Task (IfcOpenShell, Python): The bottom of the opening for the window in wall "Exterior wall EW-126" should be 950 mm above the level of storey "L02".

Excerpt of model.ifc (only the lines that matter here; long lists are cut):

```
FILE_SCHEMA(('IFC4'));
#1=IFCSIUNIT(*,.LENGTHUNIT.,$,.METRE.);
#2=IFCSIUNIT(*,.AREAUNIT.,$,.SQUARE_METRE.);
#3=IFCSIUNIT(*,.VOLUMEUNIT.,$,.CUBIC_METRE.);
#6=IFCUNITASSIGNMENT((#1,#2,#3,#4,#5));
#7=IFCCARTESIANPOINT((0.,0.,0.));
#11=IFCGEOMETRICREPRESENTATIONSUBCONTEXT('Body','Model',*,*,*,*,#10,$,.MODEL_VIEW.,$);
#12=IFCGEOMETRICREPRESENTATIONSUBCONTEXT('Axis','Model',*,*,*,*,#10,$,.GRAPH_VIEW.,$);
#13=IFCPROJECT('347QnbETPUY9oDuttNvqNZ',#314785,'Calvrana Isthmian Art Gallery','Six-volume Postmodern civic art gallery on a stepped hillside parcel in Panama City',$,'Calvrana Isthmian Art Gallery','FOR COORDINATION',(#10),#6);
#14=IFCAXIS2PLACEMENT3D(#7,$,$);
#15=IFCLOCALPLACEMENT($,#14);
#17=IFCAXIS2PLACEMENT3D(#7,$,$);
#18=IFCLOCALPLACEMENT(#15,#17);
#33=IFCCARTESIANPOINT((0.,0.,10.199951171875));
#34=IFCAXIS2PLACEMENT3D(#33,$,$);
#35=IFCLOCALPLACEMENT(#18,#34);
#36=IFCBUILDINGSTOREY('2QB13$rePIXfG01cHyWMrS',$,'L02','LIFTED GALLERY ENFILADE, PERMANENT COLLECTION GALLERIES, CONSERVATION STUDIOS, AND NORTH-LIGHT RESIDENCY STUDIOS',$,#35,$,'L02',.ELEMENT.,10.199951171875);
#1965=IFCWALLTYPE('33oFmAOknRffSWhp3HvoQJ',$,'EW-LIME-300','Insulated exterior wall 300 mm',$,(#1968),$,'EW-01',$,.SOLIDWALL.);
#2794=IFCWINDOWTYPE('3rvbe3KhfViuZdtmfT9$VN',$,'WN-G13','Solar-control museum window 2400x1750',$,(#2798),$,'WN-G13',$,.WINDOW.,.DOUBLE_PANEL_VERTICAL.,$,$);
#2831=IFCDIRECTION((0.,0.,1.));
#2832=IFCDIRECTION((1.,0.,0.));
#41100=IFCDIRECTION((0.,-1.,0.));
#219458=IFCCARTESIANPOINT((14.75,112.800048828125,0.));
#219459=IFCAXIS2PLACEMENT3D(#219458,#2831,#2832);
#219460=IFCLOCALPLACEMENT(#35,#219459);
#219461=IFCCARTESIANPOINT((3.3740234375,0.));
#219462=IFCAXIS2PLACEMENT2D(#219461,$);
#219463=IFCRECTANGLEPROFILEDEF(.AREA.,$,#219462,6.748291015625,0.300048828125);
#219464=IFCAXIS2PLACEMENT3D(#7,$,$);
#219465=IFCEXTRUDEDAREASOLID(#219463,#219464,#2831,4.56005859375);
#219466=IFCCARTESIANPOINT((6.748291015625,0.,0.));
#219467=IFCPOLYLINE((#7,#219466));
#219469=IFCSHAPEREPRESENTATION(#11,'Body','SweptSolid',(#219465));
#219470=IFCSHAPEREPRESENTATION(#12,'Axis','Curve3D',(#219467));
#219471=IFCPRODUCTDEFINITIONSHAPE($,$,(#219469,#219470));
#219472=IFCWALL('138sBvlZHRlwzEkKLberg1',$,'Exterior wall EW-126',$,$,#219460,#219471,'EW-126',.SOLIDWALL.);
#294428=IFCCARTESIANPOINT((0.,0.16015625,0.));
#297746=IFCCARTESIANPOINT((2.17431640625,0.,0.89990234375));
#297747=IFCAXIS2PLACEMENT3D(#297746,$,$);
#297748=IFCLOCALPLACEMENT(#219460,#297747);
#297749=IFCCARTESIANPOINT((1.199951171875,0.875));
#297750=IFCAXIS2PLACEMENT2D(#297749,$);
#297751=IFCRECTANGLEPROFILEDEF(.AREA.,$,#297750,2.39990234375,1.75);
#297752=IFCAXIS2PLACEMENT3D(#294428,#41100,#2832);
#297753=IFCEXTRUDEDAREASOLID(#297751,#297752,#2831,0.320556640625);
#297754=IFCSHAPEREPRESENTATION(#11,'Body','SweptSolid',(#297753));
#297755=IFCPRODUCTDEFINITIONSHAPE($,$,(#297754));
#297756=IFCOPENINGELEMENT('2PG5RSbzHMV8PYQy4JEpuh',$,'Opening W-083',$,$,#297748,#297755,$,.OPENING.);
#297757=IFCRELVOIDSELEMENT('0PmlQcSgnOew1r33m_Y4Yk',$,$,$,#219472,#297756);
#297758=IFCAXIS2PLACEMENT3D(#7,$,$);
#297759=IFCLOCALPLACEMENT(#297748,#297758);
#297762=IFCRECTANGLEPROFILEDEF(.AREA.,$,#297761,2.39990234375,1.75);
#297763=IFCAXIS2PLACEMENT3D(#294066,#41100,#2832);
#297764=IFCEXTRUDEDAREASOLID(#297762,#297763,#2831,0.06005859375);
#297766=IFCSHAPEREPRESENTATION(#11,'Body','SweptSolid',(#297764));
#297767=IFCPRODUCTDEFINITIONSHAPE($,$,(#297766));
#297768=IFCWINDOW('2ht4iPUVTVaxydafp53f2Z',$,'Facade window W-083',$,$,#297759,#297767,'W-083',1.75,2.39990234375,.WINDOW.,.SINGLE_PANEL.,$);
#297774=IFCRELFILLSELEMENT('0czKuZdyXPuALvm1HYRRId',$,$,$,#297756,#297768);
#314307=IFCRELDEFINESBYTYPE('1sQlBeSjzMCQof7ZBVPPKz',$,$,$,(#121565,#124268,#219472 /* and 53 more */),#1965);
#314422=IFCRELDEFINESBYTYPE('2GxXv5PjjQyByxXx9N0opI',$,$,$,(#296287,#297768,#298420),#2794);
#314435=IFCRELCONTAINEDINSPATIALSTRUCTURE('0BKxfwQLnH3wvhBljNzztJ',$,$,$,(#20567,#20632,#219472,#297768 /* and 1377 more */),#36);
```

```python
import numpy as np
import ifcopenshell
import ifcopenshell.api.geometry
import ifcopenshell.geom
import ifcopenshell.util.element
import ifcopenshell.util.placement
import ifcopenshell.util.shape
import ifcopenshell.util.unit

model = ifcopenshell.open("model.ifc")
unit_scale = ifcopenshell.util.unit.calculate_unit_scale(model)

window = model.by_guid("2ht4iPUVTVaxydafp53f2Z")
opening = window.FillsVoids[0].RelatingOpeningElement
storey = ifcopenshell.util.element.get_container(window, ifc_class="IfcBuildingStorey")
level = ifcopenshell.util.placement.get_local_placement(storey.ObjectPlacement)[2, 3]

# The opening's origin need not be at the sill, so measure its lowest point.
shape = ifcopenshell.geom.create_shape(ifcopenshell.geom.settings(), opening)
bottom = ifcopenshell.util.shape.get_shape_bottom_elevation(shape, shape.geometry) / unit_scale
dz = level + 0.95 / unit_scale - bottom

shift = np.array([0.0, 0.0, dz])
# The window is placed relative to its opening, so it follows when the opening moves.
matrix = ifcopenshell.util.placement.get_local_placement(opening.ObjectPlacement)
matrix[:3, 3] += shift
ifcopenshell.api.geometry.edit_object_placement(
    model, product=opening, matrix=matrix, is_si=False, should_transform_children=True
)

print(f"moved by {dz * unit_scale:+.3f} m")

model.write("model_v2.ifc")
```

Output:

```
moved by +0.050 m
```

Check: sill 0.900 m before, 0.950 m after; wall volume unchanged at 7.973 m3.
